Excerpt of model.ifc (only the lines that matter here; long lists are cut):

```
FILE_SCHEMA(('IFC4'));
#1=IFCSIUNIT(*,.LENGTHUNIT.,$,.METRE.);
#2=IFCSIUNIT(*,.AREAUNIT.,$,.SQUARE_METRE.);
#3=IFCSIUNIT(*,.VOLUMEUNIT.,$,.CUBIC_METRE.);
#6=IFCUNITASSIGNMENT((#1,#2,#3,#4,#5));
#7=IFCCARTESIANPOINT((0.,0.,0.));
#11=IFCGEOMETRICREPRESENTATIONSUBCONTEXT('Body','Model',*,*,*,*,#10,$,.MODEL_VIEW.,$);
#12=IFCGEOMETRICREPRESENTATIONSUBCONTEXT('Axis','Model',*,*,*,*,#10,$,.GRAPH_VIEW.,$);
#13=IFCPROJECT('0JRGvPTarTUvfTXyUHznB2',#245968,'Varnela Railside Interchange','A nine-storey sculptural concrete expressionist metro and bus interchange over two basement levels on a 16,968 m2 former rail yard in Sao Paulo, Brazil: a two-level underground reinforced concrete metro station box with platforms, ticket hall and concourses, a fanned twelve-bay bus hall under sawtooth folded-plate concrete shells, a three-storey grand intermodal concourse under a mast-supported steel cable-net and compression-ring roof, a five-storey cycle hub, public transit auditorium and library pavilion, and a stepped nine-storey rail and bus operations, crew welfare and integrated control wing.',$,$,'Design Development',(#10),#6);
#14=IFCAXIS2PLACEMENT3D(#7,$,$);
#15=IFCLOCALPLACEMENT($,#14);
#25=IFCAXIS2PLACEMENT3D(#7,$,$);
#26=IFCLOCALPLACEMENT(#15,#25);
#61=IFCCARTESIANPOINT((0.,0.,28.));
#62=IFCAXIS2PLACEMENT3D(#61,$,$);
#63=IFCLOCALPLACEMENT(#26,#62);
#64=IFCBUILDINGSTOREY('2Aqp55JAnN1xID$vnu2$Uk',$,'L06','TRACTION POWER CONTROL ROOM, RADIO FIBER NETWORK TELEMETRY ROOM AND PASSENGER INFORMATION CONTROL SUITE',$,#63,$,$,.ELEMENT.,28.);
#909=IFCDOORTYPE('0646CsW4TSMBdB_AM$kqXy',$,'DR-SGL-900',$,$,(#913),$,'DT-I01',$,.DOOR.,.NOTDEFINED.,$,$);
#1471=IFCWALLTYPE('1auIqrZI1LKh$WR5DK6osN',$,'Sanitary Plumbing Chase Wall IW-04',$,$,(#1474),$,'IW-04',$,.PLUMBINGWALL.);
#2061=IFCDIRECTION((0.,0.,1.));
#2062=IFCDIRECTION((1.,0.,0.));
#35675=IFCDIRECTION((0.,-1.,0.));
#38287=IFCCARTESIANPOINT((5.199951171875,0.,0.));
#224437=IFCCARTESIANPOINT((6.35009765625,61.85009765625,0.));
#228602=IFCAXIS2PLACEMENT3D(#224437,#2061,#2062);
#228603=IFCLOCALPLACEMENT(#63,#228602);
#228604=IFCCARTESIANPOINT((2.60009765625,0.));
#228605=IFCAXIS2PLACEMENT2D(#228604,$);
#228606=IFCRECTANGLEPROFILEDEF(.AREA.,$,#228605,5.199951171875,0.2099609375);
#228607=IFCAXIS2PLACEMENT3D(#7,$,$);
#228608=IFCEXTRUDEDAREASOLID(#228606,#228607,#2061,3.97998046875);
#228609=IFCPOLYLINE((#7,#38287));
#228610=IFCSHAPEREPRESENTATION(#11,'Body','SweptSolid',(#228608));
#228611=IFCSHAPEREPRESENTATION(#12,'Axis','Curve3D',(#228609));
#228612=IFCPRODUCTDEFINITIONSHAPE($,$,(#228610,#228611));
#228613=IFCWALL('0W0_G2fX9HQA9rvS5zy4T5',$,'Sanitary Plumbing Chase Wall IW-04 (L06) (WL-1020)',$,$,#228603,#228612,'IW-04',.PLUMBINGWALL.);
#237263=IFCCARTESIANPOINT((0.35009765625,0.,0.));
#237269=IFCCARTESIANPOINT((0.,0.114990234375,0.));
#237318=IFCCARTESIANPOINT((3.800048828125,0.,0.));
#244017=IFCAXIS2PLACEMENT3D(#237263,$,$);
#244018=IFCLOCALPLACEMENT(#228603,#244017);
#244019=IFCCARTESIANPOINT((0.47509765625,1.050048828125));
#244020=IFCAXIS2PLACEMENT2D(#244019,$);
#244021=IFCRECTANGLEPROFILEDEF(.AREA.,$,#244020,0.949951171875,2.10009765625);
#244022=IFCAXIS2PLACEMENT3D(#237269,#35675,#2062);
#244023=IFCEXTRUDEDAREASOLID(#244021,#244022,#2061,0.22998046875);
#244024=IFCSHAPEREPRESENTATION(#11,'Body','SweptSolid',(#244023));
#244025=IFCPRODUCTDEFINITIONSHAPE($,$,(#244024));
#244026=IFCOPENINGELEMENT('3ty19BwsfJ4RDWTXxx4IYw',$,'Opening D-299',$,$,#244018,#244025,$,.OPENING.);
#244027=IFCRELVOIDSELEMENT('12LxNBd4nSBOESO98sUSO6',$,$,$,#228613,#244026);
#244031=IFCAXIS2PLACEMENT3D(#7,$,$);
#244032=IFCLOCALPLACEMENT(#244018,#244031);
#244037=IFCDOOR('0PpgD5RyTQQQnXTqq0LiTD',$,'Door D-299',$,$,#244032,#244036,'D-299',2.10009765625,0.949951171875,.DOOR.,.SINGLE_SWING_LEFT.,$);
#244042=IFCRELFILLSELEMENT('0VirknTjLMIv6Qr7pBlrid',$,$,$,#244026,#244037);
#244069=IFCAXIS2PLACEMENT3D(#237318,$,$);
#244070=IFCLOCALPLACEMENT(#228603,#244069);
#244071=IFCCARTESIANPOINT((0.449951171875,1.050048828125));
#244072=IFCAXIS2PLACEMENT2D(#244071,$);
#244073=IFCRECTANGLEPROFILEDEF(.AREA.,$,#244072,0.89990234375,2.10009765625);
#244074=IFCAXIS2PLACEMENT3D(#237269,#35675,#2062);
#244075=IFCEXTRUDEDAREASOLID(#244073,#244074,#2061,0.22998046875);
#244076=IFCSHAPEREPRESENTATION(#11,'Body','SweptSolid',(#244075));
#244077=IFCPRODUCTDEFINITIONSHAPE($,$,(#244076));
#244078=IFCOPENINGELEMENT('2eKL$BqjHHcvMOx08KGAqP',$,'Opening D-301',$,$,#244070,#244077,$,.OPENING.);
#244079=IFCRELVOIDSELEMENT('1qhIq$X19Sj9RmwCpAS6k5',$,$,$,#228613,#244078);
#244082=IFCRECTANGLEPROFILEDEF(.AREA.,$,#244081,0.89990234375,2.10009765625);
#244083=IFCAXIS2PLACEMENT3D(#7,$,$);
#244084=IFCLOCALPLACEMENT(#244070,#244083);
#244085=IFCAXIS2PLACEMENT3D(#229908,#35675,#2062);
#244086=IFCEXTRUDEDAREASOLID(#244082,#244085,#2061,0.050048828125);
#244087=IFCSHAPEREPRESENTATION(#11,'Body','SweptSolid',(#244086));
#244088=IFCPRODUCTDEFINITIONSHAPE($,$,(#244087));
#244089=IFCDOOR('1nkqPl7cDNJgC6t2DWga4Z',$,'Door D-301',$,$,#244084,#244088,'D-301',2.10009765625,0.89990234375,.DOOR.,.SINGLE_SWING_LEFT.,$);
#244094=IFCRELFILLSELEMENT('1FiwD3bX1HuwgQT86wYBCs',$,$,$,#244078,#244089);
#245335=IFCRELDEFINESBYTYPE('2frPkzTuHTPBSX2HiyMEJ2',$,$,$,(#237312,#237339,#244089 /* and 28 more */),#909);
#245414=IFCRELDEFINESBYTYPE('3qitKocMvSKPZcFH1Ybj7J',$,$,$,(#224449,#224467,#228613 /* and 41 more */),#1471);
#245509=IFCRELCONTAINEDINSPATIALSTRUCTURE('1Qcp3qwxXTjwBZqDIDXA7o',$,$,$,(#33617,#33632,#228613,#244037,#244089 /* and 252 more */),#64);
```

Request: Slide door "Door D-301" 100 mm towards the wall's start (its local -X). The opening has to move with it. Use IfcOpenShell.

```python
import ifcopenshell
import ifcopenshell.api.geometry
import ifcopenshell.util.placement

model = ifcopenshell.open("model.ifc")

door = model.by_guid("1nkqPl7cDNJgC6t2DWga4Z")
opening = door.FillsVoids[0].RelatingOpeningElement
wall = opening.VoidsElements[0].RelatingBuildingElement

wall_matrix = ifcopenshell.util.placement.get_local_placement(wall.ObjectPlacement)
shift = wall_matrix[:3, 0] * -0.1
before = ifcopenshell.util.placement.get_local_placement(door.ObjectPlacement)[:3, 3].copy()

# The door is placed relative to its opening, so it follows when the opening moves.
matrix = ifcopenshell.util.placement.get_local_placement(opening.ObjectPlacement)
matrix[:3, 3] += shift
ifcopenshell.api.geometry.edit_object_placement(
    model, product=opening, matrix=matrix, is_si=False, should_transform_children=True
)

after = ifcopenshell.util.placement.get_local_placement(door.ObjectPlacement)[:3, 3]
print("door moved by", (after - before).round(3) + 0.0)

model.write("model-out.ifc")
```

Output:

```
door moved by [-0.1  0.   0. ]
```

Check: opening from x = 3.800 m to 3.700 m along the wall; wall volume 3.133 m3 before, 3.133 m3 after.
